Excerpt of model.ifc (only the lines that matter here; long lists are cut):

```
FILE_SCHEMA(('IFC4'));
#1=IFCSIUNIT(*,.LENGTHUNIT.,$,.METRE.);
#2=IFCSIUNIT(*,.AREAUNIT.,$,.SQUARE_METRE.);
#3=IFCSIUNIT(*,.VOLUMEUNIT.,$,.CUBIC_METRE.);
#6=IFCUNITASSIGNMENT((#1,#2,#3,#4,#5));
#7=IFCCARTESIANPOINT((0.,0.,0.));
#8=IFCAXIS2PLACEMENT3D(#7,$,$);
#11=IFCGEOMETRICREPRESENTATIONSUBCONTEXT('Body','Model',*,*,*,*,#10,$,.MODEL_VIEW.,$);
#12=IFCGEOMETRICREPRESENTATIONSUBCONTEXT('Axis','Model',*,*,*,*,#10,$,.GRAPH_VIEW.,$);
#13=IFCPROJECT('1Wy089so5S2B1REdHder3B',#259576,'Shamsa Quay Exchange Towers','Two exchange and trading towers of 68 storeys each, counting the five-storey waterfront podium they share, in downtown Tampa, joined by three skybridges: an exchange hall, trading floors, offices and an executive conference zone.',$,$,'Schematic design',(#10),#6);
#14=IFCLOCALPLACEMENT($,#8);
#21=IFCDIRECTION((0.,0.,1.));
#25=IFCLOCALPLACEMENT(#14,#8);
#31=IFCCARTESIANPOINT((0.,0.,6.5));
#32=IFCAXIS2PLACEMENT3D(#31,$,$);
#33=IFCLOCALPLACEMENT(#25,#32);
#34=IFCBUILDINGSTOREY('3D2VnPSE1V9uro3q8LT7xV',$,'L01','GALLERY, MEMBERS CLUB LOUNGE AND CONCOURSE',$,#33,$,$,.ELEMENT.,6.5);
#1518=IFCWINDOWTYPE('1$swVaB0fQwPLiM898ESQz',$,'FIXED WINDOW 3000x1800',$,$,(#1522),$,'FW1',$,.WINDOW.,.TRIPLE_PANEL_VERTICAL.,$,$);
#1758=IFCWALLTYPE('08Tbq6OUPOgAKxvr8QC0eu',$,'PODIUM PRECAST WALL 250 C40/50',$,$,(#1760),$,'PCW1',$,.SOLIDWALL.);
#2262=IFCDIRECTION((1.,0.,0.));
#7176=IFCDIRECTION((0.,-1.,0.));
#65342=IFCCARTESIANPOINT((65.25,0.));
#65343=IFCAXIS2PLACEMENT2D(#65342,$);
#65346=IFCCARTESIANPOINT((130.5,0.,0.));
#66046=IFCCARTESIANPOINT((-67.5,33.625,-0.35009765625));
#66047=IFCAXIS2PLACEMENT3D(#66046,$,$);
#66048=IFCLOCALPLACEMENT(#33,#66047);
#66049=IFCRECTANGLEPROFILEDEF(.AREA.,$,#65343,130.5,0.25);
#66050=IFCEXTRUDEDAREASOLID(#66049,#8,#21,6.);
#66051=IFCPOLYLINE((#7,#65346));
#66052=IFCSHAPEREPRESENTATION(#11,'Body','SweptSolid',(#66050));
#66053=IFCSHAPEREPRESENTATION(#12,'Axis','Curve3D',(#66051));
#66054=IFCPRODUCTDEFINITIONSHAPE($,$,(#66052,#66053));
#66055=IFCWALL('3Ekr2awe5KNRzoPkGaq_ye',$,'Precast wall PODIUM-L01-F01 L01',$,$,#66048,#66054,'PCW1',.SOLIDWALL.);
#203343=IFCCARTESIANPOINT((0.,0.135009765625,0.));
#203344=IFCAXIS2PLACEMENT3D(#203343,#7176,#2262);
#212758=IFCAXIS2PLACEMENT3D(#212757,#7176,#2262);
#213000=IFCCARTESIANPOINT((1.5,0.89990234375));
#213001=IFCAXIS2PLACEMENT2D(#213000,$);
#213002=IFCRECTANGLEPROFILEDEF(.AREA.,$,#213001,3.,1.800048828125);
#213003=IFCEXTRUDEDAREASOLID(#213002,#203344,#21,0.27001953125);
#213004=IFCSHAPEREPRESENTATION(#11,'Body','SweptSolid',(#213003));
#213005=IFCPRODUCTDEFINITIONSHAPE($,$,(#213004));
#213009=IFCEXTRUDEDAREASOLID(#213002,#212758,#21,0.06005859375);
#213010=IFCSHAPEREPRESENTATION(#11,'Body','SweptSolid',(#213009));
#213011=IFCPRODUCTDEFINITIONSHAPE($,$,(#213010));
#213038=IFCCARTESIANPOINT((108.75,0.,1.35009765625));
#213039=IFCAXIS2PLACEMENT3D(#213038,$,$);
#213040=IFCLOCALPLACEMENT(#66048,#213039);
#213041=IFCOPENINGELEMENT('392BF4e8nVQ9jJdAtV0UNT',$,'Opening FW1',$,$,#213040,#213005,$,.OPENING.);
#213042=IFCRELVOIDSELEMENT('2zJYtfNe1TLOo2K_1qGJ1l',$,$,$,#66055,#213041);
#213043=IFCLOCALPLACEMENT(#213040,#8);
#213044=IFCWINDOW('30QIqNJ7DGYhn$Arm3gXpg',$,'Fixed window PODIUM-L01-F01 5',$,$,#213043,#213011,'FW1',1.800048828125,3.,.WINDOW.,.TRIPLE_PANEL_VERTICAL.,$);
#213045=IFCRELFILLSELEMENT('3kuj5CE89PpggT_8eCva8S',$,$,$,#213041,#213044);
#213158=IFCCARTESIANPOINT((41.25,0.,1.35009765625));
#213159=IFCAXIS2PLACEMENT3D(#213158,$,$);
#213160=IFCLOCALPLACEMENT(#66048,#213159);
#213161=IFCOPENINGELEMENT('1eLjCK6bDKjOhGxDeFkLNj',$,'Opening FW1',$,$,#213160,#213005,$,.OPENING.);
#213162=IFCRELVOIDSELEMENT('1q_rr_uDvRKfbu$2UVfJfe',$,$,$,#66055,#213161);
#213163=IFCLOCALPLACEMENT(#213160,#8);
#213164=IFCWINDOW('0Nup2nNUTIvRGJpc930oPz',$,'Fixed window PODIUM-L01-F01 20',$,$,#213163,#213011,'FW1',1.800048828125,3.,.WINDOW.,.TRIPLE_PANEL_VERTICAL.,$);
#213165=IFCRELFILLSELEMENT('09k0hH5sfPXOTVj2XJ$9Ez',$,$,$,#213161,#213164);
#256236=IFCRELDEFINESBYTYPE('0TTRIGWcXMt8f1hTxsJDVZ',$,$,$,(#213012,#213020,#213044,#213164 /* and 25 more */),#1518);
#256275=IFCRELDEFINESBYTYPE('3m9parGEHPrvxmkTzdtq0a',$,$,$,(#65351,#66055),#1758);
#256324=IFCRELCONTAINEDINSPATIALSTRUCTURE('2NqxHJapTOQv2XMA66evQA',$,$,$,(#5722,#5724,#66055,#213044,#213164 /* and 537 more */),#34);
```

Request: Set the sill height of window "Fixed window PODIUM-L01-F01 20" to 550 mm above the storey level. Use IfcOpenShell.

```python
import numpy as np
import ifcopenshell
import ifcopenshell.api.geometry
import ifcopenshell.geom
import ifcopenshell.util.element
import ifcopenshell.util.placement
import ifcopenshell.util.shape
import ifcopenshell.util.unit

model = ifcopenshell.open("model.ifc")
unit_scale = ifcopenshell.util.unit.calculate_unit_scale(model)

window = model.by_id(213164)
opening = window.FillsVoids[0].RelatingOpeningElement
storey = ifcopenshell.util.element.get_container(window, ifc_class="IfcBuildingStorey")
level = ifcopenshell.util.placement.get_local_placement(storey.ObjectPlacement)[2, 3]

# The opening's origin need not be at the sill, so measure its lowest point.
shape = ifcopenshell.geom.create_shape(ifcopenshell.geom.settings(), opening)
bottom = ifcopenshell.util.shape.get_shape_bottom_elevation(shape, shape.geometry) / unit_scale
dz = level + 0.55 - bottom

shift = np.array([0.0, 0.0, dz])
# The window is placed relative to its opening, so it follows when the opening moves.
matrix = ifcopenshell.util.placement.get_local_placement(opening.ObjectPlacement)
matrix[:3, 3] += shift
ifcopenshell.api.geometry.edit_object_placement(
    model, product=opening, matrix=matrix, is_si=False, should_transform_children=True
)

print(f"moved by {dz * unit_scale:+.3f} m")

model.write("model_edited.ifc")
```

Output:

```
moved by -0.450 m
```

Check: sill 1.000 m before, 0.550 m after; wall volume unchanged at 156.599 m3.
